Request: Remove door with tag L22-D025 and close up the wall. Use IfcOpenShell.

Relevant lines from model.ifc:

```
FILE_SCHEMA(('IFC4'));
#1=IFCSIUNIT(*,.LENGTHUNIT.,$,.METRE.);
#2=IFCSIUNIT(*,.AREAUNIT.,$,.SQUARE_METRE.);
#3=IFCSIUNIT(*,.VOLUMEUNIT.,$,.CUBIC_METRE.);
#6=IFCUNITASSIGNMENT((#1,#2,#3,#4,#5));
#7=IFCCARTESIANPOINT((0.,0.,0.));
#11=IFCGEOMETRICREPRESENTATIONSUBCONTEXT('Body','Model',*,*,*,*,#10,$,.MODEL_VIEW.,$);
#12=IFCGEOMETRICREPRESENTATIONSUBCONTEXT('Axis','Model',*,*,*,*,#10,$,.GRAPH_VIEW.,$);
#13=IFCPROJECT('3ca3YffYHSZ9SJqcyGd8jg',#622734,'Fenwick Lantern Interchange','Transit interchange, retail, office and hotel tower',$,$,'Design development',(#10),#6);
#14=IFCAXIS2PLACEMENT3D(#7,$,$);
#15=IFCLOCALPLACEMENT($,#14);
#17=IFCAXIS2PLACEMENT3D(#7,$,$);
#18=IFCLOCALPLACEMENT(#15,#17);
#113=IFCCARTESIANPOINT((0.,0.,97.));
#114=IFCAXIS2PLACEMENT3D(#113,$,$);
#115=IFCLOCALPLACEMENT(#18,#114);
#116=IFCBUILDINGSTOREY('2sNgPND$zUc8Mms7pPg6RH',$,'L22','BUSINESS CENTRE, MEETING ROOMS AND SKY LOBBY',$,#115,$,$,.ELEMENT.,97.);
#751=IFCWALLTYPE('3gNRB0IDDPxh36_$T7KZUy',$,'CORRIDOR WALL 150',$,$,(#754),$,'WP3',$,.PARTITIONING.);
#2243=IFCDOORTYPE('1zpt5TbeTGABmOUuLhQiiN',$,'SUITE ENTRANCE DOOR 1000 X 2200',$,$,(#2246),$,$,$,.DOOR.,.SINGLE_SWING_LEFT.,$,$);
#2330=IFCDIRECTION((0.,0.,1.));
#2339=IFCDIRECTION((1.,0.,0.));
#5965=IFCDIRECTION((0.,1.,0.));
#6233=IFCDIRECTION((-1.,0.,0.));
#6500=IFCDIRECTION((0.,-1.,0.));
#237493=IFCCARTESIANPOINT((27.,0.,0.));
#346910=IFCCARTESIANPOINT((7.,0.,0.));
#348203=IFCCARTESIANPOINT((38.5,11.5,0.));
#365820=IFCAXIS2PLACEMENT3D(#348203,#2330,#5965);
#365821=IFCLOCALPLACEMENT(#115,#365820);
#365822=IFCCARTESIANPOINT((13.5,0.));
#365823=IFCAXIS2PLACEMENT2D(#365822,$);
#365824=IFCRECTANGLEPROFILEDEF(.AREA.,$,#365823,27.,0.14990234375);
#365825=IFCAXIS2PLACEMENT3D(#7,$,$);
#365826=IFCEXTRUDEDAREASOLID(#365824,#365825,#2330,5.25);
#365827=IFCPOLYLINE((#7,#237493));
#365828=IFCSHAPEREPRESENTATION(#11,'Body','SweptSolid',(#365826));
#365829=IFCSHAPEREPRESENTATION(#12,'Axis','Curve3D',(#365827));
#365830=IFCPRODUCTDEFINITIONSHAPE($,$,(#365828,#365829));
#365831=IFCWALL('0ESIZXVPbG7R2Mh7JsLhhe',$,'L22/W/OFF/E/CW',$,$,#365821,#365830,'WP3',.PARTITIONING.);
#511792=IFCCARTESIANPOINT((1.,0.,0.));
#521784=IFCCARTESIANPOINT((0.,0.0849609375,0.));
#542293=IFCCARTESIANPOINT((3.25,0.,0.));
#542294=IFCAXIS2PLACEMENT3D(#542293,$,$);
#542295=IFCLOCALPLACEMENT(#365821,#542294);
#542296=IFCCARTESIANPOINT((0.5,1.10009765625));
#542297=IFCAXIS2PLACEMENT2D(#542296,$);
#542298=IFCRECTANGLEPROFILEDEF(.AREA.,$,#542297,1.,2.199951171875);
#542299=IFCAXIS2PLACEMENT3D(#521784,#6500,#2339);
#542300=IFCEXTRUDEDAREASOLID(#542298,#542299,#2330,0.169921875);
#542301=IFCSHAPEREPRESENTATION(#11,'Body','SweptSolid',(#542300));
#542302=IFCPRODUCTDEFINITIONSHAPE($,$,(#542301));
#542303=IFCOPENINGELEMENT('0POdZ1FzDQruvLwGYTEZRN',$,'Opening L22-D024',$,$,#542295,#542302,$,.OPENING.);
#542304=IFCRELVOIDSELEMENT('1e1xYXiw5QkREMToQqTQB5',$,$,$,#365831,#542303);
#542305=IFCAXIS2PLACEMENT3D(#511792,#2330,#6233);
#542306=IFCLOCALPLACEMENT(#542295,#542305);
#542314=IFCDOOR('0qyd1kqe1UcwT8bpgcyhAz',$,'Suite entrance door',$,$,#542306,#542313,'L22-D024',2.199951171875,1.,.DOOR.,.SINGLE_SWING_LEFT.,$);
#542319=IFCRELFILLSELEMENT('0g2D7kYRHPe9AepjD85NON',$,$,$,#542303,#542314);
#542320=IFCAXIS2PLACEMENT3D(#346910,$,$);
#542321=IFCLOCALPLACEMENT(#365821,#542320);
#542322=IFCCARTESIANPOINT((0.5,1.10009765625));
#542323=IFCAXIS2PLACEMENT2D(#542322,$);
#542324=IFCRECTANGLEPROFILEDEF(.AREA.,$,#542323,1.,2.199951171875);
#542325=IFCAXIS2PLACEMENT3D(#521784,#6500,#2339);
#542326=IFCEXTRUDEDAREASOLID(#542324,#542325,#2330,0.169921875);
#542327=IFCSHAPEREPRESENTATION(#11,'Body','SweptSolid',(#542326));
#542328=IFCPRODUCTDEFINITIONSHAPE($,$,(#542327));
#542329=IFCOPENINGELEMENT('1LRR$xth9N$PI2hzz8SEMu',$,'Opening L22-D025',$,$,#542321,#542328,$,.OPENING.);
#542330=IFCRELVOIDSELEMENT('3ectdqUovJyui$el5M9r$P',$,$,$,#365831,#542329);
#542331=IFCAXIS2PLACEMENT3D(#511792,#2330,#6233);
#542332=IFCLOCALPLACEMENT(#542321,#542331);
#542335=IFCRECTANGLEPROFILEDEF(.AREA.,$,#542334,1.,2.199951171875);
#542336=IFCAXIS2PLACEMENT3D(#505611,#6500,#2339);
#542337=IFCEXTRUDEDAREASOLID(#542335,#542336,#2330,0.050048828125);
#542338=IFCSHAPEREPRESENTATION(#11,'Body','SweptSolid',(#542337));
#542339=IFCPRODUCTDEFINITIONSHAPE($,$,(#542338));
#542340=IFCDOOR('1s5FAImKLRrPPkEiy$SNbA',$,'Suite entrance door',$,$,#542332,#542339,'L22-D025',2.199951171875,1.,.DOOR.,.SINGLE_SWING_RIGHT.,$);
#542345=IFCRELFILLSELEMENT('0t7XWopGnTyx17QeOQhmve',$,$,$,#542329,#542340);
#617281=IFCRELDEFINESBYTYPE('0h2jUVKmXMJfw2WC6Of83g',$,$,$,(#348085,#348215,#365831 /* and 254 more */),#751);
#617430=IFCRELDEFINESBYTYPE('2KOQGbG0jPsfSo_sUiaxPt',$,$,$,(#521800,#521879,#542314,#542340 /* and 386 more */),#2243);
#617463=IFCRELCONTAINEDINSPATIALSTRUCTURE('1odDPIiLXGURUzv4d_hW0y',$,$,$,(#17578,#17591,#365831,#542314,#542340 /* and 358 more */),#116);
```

```python
import ifcopenshell
import ifcopenshell.api.feature
import ifcopenshell.api.root
import ifcopenshell.geom
import ifcopenshell.util.shape

model = ifcopenshell.open("model.ifc")
settings = ifcopenshell.geom.settings()


def volume(element):
    """Net volume in cubic metres, openings subtracted."""
    shape = ifcopenshell.geom.create_shape(settings, element)
    return ifcopenshell.util.shape.get_volume(shape.geometry)


door = model.by_id(542340)
opening = door.FillsVoids[0].RelatingOpeningElement
wall = opening.VoidsElements[0].RelatingBuildingElement
before = volume(wall)

ifcopenshell.api.root.remove_product(model, product=door)
ifcopenshell.api.feature.remove_feature(model, feature=opening)

after = volume(wall)

print(f"wall volume {before:.3f} -> {after:.3f} m3")

model.write("model_v2.ifc")
```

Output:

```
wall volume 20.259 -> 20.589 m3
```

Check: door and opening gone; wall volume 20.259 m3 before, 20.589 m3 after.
